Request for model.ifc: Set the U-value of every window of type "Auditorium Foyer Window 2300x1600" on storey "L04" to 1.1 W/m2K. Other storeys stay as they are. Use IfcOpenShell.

First a look at what the model holds.

```python
import ifcopenshell
import ifcopenshell.util.element

model = ifcopenshell.open("model.ifc")
print(model.schema)
storey = next(s for s in model.by_type("IfcBuildingStorey") if s.Name == "L04")
windows = [e for e in ifcopenshell.util.element.get_decomposition(storey) if e.is_a("IfcWindow")]
seen = {}
for e in windows:
    element_type = ifcopenshell.util.element.get_type(e)
    key = (element_type.Name if element_type != e and element_type else None, ifcopenshell.util.element.get_pset(e, "Pset_WindowCommon", "ThermalTransmittance"))
    seen[key] = seen.get(key, 0) + 1
for (name, value), count in sorted(seen.items(), key=str):
    print(count, "x", name, "|", value)
```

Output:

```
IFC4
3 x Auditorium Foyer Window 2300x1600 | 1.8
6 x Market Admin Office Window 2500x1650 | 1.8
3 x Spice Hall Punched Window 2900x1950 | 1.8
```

```python
import ifcopenshell
import ifcopenshell.api.pset
import ifcopenshell.util.element

model = ifcopenshell.open("model.ifc")

storey = next(s for s in model.by_type("IfcBuildingStorey") if s.Name == "L04")
windows = [e for e in ifcopenshell.util.element.get_decomposition(storey) if e.is_a("IfcWindow")]

count = 0
for e in windows:
    element_type = ifcopenshell.util.element.get_type(e)
    if element_type in (None, e) or element_type.Name != "Auditorium Foyer Window 2300x1600":
        continue
    # add_pset returns the element's existing set when there is one.
    pset = ifcopenshell.api.pset.add_pset(model, product=e, name="Pset_WindowCommon")
    ifcopenshell.api.pset.edit_pset(model, pset=pset, properties={"ThermalTransmittance": 1.1})
    count += 1

print(count, "windows updated")

model.write("model_v2.ifc")
```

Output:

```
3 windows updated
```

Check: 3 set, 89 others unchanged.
